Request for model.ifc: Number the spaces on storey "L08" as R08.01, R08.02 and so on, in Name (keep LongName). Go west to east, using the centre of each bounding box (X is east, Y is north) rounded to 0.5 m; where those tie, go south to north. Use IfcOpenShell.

First a look at what the model holds.

```python
import ifcopenshell
import ifcopenshell.util.element
import ifcopenshell.util.placement

model = ifcopenshell.open("model.ifc")
print(model.schema)
storey = next(s for s in model.by_type("IfcBuildingStorey") if s.Name == "L08")
spaces = [e for e in ifcopenshell.util.element.get_decomposition(storey) if e.is_a("IfcSpace")]
for e in sorted(spaces, key=lambda e: e.id()):
    origin = ifcopenshell.util.placement.get_local_placement(e.ObjectPlacement)[:3, 3]
    print(e.id(), e.Name, e.LongName, origin.round(2) + 0.0, sep=" | ")
```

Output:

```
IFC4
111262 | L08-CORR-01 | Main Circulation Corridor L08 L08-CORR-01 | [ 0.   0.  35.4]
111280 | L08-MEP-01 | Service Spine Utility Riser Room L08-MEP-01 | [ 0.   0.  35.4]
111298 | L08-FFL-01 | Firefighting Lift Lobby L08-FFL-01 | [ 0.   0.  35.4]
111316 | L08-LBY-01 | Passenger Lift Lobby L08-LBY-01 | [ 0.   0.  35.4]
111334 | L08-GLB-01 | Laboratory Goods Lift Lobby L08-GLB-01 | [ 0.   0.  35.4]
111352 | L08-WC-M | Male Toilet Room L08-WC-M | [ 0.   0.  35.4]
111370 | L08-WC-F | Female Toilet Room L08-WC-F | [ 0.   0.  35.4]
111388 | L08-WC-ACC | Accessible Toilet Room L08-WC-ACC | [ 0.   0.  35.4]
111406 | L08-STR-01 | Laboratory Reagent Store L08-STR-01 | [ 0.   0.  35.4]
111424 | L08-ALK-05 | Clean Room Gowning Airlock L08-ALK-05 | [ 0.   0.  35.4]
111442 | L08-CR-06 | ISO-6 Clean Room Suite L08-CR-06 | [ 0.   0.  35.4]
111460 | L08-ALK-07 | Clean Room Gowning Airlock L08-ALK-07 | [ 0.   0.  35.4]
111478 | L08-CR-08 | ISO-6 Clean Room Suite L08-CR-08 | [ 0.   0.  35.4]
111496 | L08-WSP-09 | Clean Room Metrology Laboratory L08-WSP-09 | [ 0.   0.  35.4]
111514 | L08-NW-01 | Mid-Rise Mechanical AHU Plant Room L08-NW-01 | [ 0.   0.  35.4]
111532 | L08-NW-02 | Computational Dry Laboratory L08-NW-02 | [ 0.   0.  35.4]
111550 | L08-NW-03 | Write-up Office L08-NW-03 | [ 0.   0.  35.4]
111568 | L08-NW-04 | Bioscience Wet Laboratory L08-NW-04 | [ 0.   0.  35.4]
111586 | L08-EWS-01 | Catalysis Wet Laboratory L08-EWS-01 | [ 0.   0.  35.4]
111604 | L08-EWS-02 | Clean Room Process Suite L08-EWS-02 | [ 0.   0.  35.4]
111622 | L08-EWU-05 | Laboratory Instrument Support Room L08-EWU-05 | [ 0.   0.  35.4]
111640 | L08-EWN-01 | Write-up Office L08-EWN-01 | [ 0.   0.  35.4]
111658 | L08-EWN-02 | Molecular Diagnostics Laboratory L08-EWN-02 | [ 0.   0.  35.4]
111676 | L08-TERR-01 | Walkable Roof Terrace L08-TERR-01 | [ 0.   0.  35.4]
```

```python
import ifcopenshell
import ifcopenshell.geom
import ifcopenshell.util.element
import ifcopenshell.util.shape

model = ifcopenshell.open("model.ifc")
settings = ifcopenshell.geom.settings()
settings.set("use-world-coords", True)


def centre(element):
    shape = ifcopenshell.geom.create_shape(settings, element)
    return ifcopenshell.util.shape.get_bbox_centroid(shape.geometry)


storey = next(s for s in model.by_type("IfcBuildingStorey") if s.Name == "L08")
spaces = [e for e in ifcopenshell.util.element.get_decomposition(storey) if e.is_a("IfcSpace")]

# Insertion points can sit at a corner or the storey origin, so sort by the geometry (in metres).
centres = {e: centre(e) for e in spaces}
spaces.sort(key=lambda e: (round(centres[e][0] / 0.5), centres[e][1]))

for i, e in enumerate(spaces, start=1):
    number = f"R08.{i:02d}"
    e.Name = number
    print(e.id(), number)

model.write("model-out.ifc")
```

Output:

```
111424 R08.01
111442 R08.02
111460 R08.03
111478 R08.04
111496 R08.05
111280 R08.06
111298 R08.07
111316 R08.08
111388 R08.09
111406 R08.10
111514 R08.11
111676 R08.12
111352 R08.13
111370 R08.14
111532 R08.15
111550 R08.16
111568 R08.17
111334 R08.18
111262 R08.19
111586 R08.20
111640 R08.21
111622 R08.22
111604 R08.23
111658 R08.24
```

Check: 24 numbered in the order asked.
